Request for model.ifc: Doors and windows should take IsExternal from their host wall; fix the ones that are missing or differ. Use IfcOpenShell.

First a look at what the model holds.

```python
import ifcopenshell
import ifcopenshell.util.element

model = ifcopenshell.open("model.ifc")
print(model.schema)
seen = {}
for e in model.by_type("IfcDoor") + model.by_type("IfcWindow"):
    if not e.FillsVoids:
        continue
    host = e.FillsVoids[0].RelatingOpeningElement.VoidsElements[0].RelatingBuildingElement
    own = ifcopenshell.util.element.get_pset(e, f"Pset_{e.is_a()[3:].removesuffix('StandardCase')}Common", "IsExternal")
    wall = ifcopenshell.util.element.get_pset(host, "Pset_WallCommon", "IsExternal")
    seen[e.is_a(), own, wall] = seen.get((e.is_a(), own, wall), 0) + 1
for (cls, own, wall), count in sorted(seen.items(), key=str):
    print(count, cls, "IsExternal:", own, "| host wall:", wall)
```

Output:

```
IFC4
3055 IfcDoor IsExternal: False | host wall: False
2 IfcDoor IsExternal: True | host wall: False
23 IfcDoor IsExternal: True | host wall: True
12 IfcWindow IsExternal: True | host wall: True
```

```python
import ifcopenshell
import ifcopenshell.api.pset
import ifcopenshell.util.element

model = ifcopenshell.open("model.ifc")

count = 0
for ifc_class, pset_name in (("IfcDoor", "Pset_DoorCommon"), ("IfcWindow", "Pset_WindowCommon")):
    for e in model.by_type(ifc_class):
        if not e.FillsVoids:
            continue
        host = e.FillsVoids[0].RelatingOpeningElement.VoidsElements[0].RelatingBuildingElement
        external = ifcopenshell.util.element.get_pset(host, "Pset_WallCommon", "IsExternal")
        if external is None or ifcopenshell.util.element.get_pset(e, pset_name, "IsExternal") == external:
            continue
        pset = ifcopenshell.api.pset.add_pset(model, product=e, name=pset_name)
        ifcopenshell.api.pset.edit_pset(model, pset=pset, properties={"IsExternal": external})
        count += 1

print(count, "updated")

model.write("model_rev.ifc")
```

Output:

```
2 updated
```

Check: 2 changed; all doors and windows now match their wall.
